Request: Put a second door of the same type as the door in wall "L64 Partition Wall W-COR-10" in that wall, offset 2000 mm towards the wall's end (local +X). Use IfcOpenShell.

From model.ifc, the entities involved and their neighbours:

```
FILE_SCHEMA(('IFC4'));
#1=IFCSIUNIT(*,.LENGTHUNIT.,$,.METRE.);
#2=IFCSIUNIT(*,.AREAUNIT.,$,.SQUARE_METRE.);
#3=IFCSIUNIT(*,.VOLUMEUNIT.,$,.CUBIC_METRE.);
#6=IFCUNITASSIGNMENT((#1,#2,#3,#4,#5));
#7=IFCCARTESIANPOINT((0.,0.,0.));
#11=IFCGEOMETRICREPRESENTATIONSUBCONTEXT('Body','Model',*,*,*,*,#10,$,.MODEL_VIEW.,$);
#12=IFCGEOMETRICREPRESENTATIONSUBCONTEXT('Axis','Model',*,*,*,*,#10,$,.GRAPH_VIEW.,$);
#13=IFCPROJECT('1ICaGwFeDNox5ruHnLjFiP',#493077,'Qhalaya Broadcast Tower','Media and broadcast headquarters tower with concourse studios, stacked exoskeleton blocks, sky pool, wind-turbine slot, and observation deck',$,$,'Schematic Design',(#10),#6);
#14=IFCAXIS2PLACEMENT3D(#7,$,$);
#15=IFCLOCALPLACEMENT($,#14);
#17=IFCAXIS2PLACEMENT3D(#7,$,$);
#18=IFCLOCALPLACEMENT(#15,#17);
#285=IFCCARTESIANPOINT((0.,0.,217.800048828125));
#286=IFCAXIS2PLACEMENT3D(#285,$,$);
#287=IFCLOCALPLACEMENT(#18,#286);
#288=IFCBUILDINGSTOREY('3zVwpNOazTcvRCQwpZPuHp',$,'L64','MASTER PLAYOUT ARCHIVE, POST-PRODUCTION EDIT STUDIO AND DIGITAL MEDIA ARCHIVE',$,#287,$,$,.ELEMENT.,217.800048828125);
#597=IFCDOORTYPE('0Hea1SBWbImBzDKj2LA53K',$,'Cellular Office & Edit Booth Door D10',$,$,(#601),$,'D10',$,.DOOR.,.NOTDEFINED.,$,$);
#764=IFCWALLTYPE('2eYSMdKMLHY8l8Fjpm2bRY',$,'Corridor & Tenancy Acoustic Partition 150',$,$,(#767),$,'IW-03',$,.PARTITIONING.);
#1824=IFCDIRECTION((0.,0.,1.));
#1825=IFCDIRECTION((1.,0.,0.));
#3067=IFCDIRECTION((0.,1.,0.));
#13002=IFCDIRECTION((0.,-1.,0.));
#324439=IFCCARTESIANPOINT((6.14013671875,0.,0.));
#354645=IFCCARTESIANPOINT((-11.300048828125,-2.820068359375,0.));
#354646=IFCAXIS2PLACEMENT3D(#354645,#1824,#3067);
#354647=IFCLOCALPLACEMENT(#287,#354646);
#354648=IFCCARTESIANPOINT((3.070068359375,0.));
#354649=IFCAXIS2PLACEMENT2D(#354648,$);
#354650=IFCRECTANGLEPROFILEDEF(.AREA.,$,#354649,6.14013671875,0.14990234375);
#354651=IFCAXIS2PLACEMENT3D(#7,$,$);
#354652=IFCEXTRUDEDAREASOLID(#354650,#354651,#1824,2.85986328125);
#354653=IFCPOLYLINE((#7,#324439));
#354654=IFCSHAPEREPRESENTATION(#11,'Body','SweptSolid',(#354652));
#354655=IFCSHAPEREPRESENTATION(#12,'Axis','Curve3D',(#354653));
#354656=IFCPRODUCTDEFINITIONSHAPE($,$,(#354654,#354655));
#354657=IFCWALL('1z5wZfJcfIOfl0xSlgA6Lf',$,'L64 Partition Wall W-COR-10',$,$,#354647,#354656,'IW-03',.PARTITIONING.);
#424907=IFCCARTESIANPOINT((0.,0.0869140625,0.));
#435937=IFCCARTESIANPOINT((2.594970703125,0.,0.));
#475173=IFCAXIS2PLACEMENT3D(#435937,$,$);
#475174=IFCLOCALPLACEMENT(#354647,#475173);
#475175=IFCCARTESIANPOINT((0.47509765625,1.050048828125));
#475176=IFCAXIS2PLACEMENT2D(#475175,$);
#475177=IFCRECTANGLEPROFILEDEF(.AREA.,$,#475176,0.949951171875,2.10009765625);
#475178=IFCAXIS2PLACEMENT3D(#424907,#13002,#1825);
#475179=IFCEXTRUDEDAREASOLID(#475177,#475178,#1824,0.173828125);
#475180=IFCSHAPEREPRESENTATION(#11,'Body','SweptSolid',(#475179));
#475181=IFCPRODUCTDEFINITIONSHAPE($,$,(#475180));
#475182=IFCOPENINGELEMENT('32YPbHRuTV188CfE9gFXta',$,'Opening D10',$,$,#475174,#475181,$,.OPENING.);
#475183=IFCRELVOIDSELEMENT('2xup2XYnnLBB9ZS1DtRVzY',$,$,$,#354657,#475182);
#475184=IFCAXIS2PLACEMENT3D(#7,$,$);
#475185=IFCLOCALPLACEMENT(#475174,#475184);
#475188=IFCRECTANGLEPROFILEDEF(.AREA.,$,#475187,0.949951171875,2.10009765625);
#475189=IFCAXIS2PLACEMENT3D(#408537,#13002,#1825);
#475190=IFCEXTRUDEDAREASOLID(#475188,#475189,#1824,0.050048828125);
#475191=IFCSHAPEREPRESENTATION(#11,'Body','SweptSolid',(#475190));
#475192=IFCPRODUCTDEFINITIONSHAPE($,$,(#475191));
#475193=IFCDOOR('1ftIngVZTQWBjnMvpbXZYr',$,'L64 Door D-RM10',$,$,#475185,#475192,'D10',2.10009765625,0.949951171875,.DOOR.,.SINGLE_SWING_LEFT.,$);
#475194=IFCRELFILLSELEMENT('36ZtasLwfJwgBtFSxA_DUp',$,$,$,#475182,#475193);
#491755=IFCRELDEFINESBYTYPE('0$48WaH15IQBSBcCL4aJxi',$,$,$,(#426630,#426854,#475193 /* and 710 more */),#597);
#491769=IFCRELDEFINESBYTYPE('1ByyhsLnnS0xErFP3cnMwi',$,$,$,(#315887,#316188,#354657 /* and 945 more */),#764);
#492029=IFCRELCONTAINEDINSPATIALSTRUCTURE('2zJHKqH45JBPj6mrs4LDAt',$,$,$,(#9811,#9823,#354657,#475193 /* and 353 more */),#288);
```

```python
import ifcopenshell
import ifcopenshell.api.feature
import ifcopenshell.api.geometry
import ifcopenshell.api.root
import ifcopenshell.geom
import ifcopenshell.util.element
import ifcopenshell.util.placement
import ifcopenshell.util.shape

model = ifcopenshell.open("model.ifc")
settings = ifcopenshell.geom.settings()


def volume(element):
    """Net volume in cubic metres, openings subtracted."""
    shape = ifcopenshell.geom.create_shape(settings, element)
    return ifcopenshell.util.shape.get_volume(shape.geometry)


door = model.by_guid("1ftIngVZTQWBjnMvpbXZYr")
opening = door.FillsVoids[0].RelatingOpeningElement
wall = opening.VoidsElements[0].RelatingBuildingElement
before = volume(wall)
shift = ifcopenshell.util.placement.get_local_placement(wall.ObjectPlacement)[:3, 0] * 2.0

# copy_class copies the void relationship, type, container and properties, but no geometry.
new_opening = ifcopenshell.api.root.copy_class(model, product=opening)
new_opening.Representation = ifcopenshell.util.element.copy_deep(
    model, opening.Representation, exclude=["IfcGeometricRepresentationContext", "IfcRepresentationMap"]
)
new_door = ifcopenshell.api.root.copy_class(model, product=door)
new_door.Representation = ifcopenshell.util.element.copy_deep(
    model, door.Representation, exclude=["IfcGeometricRepresentationContext", "IfcRepresentationMap"]
)
new_door.Tag = None
ifcopenshell.api.feature.add_filling(model, opening=new_opening, element=new_door)

for old, new in ((opening, new_opening), (door, new_door)):
    matrix = ifcopenshell.util.placement.get_local_placement(old.ObjectPlacement)
    matrix[:3, 3] += shift
    ifcopenshell.api.geometry.edit_object_placement(model, product=new, matrix=matrix, is_si=False)

after = volume(wall)

print(f"wall volume {before:.3f} -> {after:.3f} m3")

model.write("model-out.ifc")
```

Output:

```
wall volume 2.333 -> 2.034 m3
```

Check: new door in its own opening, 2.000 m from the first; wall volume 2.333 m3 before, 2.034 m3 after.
